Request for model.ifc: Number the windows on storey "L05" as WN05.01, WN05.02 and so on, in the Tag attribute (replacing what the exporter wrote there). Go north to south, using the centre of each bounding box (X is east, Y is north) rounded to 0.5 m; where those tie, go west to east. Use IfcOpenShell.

First a look at what the model holds.

```python
import ifcopenshell
import ifcopenshell.util.element
import ifcopenshell.util.placement

model = ifcopenshell.open("model.ifc")
print(model.schema)
storey = next(s for s in model.by_type("IfcBuildingStorey") if s.Name == "L05")
windows = [e for e in ifcopenshell.util.element.get_decomposition(storey) if e.is_a("IfcWindow")]
for e in sorted(windows, key=lambda e: e.id()):
    origin = ifcopenshell.util.placement.get_local_placement(e.ObjectPlacement)[:3, 3]
    print(e.id(), e.Tag, e.Name, origin.round(2) + 0.0, sep=" | ")
```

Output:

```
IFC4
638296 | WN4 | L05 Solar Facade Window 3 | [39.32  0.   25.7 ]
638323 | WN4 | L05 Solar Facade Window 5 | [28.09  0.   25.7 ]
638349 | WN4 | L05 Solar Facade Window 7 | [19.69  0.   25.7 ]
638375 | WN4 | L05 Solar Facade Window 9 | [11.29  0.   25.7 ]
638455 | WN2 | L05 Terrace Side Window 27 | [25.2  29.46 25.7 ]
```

```python
import ifcopenshell
import ifcopenshell.geom
import ifcopenshell.util.element
import ifcopenshell.util.shape

model = ifcopenshell.open("model.ifc")
settings = ifcopenshell.geom.settings()
settings.set("use-world-coords", True)


def centre(element):
    shape = ifcopenshell.geom.create_shape(settings, element)
    return ifcopenshell.util.shape.get_bbox_centroid(shape.geometry)


storey = next(s for s in model.by_type("IfcBuildingStorey") if s.Name == "L05")
windows = [e for e in ifcopenshell.util.element.get_decomposition(storey) if e.is_a("IfcWindow")]

# Insertion points can sit at a corner or the storey origin, so sort by the geometry (in metres).
centres = {e: centre(e) for e in windows}
windows.sort(key=lambda e: (-round(centres[e][1] / 0.5), centres[e][0]))

for i, e in enumerate(windows, start=1):
    number = f"WN05.{i:02d}"
    e.Tag = number
    print(e.id(), number)

model.write("model_v2.ifc")
```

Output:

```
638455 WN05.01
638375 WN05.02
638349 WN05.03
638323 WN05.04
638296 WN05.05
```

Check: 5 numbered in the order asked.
